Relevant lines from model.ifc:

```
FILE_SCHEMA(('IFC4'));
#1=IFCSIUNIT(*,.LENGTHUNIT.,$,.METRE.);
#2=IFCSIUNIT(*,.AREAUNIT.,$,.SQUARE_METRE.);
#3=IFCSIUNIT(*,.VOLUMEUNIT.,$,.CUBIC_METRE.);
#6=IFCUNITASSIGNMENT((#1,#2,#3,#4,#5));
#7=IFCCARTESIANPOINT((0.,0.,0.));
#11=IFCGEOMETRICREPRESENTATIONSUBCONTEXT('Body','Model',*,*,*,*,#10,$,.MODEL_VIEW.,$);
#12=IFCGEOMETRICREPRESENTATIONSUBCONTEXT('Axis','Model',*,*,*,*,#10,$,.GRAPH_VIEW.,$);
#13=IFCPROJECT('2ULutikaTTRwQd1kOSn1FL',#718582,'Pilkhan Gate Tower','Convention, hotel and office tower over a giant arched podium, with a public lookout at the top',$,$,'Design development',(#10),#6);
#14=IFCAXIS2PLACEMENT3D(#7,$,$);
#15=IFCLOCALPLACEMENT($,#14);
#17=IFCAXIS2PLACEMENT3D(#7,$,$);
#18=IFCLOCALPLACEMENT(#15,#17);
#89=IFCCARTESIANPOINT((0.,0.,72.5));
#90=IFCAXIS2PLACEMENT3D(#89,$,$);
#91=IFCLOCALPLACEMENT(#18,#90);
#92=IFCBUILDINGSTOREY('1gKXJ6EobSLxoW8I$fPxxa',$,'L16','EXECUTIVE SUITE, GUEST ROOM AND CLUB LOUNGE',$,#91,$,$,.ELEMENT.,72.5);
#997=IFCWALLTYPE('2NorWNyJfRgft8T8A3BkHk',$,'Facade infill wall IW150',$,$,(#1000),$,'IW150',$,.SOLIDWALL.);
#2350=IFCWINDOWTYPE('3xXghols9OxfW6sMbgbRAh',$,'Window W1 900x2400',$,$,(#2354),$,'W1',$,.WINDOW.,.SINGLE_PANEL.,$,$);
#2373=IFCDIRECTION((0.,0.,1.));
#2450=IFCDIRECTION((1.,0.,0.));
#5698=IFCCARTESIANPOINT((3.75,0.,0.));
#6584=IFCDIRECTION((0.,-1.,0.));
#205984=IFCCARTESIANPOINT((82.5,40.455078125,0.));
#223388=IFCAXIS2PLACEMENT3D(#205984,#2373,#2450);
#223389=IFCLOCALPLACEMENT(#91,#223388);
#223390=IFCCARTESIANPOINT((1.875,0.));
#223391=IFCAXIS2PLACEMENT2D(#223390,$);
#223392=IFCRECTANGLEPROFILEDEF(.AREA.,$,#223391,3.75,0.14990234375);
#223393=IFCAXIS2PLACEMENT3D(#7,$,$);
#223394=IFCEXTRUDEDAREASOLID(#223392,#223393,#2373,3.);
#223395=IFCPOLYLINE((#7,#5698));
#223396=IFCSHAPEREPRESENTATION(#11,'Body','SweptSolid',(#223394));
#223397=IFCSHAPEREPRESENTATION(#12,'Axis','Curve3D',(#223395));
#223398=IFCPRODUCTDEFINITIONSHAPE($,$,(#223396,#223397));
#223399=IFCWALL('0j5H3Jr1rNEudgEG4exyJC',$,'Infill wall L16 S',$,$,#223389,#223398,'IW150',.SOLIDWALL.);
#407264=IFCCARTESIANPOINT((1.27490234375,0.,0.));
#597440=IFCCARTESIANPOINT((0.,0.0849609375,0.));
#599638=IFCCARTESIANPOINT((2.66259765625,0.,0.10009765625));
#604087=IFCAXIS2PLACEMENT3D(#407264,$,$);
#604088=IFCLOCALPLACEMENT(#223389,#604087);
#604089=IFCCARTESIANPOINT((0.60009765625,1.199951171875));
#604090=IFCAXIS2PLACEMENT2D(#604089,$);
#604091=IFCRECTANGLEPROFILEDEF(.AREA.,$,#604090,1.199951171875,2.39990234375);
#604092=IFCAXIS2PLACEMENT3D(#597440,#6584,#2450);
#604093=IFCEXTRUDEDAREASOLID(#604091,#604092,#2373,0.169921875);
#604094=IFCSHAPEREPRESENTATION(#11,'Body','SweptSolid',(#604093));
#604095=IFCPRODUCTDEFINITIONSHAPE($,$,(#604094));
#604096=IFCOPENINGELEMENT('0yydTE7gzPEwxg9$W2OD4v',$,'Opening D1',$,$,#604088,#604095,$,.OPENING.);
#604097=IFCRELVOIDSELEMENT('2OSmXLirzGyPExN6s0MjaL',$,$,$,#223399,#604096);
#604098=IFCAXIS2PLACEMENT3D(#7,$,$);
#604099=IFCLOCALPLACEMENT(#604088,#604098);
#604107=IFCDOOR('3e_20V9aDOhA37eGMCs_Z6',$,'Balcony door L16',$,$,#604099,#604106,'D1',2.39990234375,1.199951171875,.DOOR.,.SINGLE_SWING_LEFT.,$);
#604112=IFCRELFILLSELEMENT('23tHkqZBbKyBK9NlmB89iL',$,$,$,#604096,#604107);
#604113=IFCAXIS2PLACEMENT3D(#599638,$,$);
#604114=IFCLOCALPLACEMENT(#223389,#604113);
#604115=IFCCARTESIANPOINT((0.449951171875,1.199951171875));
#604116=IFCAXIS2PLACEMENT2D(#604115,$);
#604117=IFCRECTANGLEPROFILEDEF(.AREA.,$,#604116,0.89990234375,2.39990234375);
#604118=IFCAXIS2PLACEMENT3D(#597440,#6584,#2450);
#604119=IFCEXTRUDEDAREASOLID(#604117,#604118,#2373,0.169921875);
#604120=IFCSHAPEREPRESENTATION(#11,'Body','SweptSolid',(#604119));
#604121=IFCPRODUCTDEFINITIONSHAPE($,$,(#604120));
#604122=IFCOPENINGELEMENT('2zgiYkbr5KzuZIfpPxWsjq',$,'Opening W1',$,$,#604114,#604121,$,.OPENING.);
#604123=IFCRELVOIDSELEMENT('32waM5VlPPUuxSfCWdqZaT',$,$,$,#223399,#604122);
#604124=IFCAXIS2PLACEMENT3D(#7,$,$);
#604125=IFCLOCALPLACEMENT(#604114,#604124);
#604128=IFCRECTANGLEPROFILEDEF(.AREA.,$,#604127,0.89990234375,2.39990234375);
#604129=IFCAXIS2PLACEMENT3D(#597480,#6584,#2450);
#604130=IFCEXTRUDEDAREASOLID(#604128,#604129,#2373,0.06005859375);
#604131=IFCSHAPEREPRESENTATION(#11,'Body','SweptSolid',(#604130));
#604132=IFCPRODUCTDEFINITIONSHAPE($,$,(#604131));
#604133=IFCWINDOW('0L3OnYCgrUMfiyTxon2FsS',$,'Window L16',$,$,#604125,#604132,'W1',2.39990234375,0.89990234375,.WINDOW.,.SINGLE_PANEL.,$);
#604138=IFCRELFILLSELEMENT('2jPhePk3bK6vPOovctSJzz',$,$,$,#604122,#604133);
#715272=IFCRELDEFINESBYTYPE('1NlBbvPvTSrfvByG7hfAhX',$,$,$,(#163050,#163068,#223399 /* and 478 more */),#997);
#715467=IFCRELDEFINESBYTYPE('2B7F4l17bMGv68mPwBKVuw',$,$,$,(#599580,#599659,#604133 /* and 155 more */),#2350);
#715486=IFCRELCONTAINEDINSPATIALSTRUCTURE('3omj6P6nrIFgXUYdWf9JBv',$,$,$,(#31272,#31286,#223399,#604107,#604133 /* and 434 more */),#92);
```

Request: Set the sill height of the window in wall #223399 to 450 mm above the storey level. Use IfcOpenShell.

```python
import numpy as np
import ifcopenshell
import ifcopenshell.api.geometry
import ifcopenshell.geom
import ifcopenshell.util.element
import ifcopenshell.util.placement
import ifcopenshell.util.shape
import ifcopenshell.util.unit

model = ifcopenshell.open("model.ifc")
unit_scale = ifcopenshell.util.unit.calculate_unit_scale(model)

window = model.by_id(604133)
opening = window.FillsVoids[0].RelatingOpeningElement
storey = ifcopenshell.util.element.get_container(window, ifc_class="IfcBuildingStorey")
level = ifcopenshell.util.placement.get_local_placement(storey.ObjectPlacement)[2, 3]

# The opening's origin need not be at the sill, so measure its lowest point.
shape = ifcopenshell.geom.create_shape(ifcopenshell.geom.settings(), opening)
bottom = ifcopenshell.util.shape.get_shape_bottom_elevation(shape, shape.geometry) / unit_scale
dz = level + 0.45 - bottom

shift = np.array([0.0, 0.0, dz])
# The window is placed relative to its opening, so it follows when the opening moves.
matrix = ifcopenshell.util.placement.get_local_placement(opening.ObjectPlacement)
matrix[:3, 3] += shift
ifcopenshell.api.geometry.edit_object_placement(
    model, product=opening, matrix=matrix, is_si=False, should_transform_children=True
)

print(f"moved by {dz * unit_scale:+.3f} m")

model.write("model_edited.ifc")
```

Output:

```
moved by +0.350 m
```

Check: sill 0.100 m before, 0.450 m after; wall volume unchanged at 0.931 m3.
